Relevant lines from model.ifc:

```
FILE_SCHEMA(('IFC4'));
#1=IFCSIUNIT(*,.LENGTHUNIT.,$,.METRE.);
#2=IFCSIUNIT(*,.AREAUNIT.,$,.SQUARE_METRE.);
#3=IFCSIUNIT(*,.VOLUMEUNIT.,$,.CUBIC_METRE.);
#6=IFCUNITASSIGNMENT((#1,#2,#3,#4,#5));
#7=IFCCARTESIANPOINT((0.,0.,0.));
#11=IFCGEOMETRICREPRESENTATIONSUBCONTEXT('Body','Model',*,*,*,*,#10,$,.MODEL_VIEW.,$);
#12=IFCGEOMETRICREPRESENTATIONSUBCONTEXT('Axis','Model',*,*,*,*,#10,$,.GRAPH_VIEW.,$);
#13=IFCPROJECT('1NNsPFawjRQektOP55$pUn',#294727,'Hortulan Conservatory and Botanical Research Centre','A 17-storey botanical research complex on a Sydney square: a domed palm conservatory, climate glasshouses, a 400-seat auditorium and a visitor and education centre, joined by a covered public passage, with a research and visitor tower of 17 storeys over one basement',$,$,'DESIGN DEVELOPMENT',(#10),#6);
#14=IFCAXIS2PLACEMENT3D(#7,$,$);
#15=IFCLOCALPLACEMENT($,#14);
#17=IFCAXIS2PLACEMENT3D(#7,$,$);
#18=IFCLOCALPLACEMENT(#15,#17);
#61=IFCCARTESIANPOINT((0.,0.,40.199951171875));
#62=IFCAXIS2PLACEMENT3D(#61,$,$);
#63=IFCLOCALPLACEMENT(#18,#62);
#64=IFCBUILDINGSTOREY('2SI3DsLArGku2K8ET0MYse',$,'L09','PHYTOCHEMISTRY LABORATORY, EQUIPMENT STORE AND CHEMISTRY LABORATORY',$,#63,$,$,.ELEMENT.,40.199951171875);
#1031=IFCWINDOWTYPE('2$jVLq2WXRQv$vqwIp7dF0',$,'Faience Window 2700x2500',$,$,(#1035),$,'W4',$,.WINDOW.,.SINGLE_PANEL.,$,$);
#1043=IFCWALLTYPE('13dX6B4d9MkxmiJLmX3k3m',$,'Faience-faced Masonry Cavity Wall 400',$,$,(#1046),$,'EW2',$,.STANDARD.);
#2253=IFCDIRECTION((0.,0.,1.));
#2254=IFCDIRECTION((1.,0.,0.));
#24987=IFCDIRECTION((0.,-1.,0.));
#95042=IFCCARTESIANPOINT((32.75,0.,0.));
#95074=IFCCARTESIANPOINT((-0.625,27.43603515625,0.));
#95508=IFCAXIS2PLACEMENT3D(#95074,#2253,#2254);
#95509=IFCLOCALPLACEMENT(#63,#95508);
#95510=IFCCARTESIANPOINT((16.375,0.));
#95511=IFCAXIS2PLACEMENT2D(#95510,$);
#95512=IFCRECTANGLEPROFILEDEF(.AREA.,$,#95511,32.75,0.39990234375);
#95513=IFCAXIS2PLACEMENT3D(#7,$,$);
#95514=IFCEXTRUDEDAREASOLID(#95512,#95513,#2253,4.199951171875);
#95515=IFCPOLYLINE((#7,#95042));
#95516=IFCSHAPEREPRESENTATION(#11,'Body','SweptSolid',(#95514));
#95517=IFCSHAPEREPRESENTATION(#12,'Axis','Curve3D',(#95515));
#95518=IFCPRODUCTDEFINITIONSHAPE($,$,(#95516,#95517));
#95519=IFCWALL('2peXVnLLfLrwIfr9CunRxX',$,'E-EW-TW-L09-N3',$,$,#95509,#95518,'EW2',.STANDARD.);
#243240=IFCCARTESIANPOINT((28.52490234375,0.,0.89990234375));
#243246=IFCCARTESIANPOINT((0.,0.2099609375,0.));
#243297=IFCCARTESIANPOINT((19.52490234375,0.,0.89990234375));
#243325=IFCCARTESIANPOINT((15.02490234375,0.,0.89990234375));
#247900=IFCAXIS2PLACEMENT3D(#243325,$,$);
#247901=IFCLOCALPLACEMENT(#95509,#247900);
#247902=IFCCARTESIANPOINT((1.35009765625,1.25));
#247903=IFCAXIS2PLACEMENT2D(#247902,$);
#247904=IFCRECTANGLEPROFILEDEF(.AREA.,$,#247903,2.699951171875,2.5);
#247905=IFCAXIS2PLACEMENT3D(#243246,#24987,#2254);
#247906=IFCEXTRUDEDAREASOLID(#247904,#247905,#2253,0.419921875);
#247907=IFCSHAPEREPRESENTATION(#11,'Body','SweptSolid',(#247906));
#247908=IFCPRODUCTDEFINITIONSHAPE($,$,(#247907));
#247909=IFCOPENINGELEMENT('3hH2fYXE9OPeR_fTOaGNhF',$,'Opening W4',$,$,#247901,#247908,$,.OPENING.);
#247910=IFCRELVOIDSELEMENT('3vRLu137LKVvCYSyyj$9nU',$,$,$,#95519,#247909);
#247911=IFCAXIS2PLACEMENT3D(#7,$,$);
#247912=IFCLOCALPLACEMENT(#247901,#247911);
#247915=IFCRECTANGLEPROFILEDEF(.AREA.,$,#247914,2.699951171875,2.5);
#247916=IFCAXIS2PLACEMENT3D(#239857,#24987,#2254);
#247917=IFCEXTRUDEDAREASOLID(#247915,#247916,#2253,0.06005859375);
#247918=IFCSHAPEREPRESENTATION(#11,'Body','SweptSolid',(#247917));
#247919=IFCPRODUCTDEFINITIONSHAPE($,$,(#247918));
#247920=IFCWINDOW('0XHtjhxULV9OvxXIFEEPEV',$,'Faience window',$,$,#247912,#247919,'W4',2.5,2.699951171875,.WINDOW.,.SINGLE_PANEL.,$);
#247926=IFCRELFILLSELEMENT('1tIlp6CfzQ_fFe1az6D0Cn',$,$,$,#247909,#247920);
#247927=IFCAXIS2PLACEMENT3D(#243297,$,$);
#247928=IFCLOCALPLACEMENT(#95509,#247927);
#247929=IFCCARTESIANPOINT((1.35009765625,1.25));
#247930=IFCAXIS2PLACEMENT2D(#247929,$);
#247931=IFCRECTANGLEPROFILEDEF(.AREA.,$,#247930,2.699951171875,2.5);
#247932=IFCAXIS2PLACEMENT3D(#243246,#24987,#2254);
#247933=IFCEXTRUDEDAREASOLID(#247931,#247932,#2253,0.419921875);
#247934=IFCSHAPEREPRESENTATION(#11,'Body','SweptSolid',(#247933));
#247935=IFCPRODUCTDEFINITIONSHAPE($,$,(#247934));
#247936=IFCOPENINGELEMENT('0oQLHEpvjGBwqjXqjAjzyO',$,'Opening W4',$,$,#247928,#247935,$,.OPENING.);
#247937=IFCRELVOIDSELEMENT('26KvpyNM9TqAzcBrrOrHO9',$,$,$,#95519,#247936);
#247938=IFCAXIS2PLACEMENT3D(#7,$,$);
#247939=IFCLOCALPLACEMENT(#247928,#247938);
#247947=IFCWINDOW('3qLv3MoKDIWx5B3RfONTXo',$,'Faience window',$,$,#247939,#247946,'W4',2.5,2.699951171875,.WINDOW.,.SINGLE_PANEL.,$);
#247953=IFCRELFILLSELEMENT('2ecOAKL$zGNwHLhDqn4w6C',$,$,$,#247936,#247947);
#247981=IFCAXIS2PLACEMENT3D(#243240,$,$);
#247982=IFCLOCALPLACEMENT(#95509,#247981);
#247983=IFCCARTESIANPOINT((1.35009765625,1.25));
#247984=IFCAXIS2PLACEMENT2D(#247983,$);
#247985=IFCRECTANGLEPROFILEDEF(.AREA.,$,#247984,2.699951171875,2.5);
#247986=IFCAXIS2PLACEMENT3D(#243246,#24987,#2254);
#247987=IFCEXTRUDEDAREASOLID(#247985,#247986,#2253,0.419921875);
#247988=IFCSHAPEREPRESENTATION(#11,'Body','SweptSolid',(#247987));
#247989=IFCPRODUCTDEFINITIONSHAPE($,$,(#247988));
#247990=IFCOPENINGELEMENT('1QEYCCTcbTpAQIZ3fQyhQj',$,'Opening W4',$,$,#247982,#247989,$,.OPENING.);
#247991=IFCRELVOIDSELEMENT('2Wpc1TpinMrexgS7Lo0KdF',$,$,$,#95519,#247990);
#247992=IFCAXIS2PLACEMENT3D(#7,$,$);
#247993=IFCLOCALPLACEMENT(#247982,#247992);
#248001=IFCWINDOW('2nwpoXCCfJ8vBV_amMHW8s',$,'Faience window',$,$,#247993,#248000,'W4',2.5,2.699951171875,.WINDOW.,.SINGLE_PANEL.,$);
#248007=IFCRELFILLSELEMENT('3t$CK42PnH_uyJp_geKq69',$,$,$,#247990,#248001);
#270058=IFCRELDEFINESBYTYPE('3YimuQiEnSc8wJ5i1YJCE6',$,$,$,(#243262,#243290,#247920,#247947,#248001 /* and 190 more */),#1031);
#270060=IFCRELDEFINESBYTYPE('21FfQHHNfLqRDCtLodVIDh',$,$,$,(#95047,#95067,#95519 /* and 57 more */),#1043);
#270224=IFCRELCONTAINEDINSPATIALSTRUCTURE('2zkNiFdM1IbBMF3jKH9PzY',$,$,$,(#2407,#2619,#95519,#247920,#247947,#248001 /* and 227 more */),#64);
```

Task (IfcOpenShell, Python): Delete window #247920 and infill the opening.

```python
import ifcopenshell
import ifcopenshell.api.feature
import ifcopenshell.api.root
import ifcopenshell.geom
import ifcopenshell.util.shape

model = ifcopenshell.open("model.ifc")
settings = ifcopenshell.geom.settings()


def volume(element):
    """Net volume in cubic metres, openings subtracted."""
    shape = ifcopenshell.geom.create_shape(settings, element)
    return ifcopenshell.util.shape.get_volume(shape.geometry)


window = model.by_id(247920)
opening = window.FillsVoids[0].RelatingOpeningElement
wall = opening.VoidsElements[0].RelatingBuildingElement
before = volume(wall)

ifcopenshell.api.root.remove_product(model, product=window)
ifcopenshell.api.feature.remove_feature(model, feature=opening)

after = volume(wall)

print(f"wall volume {before:.3f} -> {after:.3f} m3")

model.write("model_edited.ifc")
```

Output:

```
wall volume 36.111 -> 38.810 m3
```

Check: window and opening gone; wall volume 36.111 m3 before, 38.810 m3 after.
